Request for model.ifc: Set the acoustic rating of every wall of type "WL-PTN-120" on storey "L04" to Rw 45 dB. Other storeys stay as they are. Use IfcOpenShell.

First a look at what the model holds.

```python
import ifcopenshell
import ifcopenshell.util.element

model = ifcopenshell.open("model.ifc")
print(model.schema)
storey = next(s for s in model.by_type("IfcBuildingStorey") if s.Name == "L04")
walls = [e for e in ifcopenshell.util.element.get_decomposition(storey) if e.is_a("IfcWall")]
seen = {}
for e in walls:
    element_type = ifcopenshell.util.element.get_type(e)
    key = (element_type.Name if element_type != e and element_type else None, ifcopenshell.util.element.get_pset(e, "Pset_WallCommon", "AcousticRating"))
    seen[key] = seen.get(key, 0) + 1
for (name, value), count in sorted(seen.items(), key=str):
    print(count, "x", name, "|", value)
```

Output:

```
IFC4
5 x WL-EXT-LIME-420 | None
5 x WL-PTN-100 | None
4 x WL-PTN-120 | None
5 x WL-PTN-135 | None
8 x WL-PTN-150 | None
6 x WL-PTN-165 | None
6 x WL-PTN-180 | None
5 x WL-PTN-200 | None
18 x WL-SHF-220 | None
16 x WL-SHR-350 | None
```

```python
import ifcopenshell
import ifcopenshell.api.pset
import ifcopenshell.util.element

model = ifcopenshell.open("model.ifc")

storey = next(s for s in model.by_type("IfcBuildingStorey") if s.Name == "L04")
walls = [e for e in ifcopenshell.util.element.get_decomposition(storey) if e.is_a("IfcWall")]

count = 0
for e in walls:
    element_type = ifcopenshell.util.element.get_type(e)
    if element_type in (None, e) or element_type.Name != "WL-PTN-120":
        continue
    # add_pset returns the element's existing set when there is one.
    pset = ifcopenshell.api.pset.add_pset(model, product=e, name="Pset_WallCommon")
    ifcopenshell.api.pset.edit_pset(model, pset=pset, properties={"AcousticRating": "Rw 45 dB"})
    count += 1

print(count, "walls updated")

model.write("model_rev.ifc")
```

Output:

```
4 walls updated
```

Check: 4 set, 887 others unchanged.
